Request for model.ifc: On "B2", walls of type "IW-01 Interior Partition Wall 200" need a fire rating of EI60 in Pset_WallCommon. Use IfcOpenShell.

First a look at what the model holds.

```python
import ifcopenshell
import ifcopenshell.util.element

model = ifcopenshell.open("model.ifc")
print(model.schema)
storey = next(s for s in model.by_type("IfcBuildingStorey") if s.Name == "B2")
walls = [e for e in ifcopenshell.util.element.get_decomposition(storey) if e.is_a("IfcWall")]
seen = {}
for e in walls:
    element_type = ifcopenshell.util.element.get_type(e)
    key = (element_type.Name if element_type != e and element_type else None, ifcopenshell.util.element.get_pset(e, "Pset_WallCommon", "FireRating"))
    seen[key] = seen.get(key, 0) + 1
for (name, value), count in sorted(seen.items(), key=str):
    print(count, "x", name, "|", value)
```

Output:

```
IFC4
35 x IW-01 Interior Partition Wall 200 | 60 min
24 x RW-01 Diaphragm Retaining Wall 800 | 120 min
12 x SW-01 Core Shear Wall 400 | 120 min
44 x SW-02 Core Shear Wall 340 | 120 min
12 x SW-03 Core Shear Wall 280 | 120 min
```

```python
import ifcopenshell
import ifcopenshell.api.pset
import ifcopenshell.util.element

model = ifcopenshell.open("model.ifc")

storey = next(s for s in model.by_type("IfcBuildingStorey") if s.Name == "B2")
walls = [e for e in ifcopenshell.util.element.get_decomposition(storey) if e.is_a("IfcWall")]

count = 0
for e in walls:
    element_type = ifcopenshell.util.element.get_type(e)
    if element_type in (None, e) or element_type.Name != "IW-01 Interior Partition Wall 200":
        continue
    # add_pset returns the element's existing set when there is one.
    pset = ifcopenshell.api.pset.add_pset(model, product=e, name="Pset_WallCommon")
    ifcopenshell.api.pset.edit_pset(model, pset=pset, properties={"FireRating": "EI60"})
    count += 1

print(count, "walls updated")

model.write("model_v2.ifc")
```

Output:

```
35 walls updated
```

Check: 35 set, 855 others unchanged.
